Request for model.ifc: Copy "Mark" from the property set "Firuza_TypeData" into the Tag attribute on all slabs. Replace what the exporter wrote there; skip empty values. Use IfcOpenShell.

First a look at what the model holds.

```python
import ifcopenshell
import ifcopenshell.util.element

model = ifcopenshell.open("model.ifc")
print(model.schema)
slabs = model.by_type("IfcSlab")
print(len(slabs), "slabs")
for e in slabs[:8]:
    source = ifcopenshell.util.element.get_pset(e, "Firuza_TypeData", "Mark")
    target = e.Tag
    print(e.id(), repr(source), repr(target), sep=" | ")
```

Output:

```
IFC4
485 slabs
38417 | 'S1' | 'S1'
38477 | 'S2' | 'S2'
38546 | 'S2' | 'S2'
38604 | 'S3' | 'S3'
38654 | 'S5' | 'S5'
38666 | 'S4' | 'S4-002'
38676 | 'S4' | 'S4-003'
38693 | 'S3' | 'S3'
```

```python
import ifcopenshell
import ifcopenshell.util.element

model = ifcopenshell.open("model.ifc")

count = 0
for e in model.by_type("IfcSlab"):
    value = ifcopenshell.util.element.get_pset(e, "Firuza_TypeData", "Mark")
    current = e.Tag
    if not value or not value.strip() or current == value:
        continue
    e.Tag = value
    count += 1

print(count, "slabs updated")

model.write("model_updated.ifc")
```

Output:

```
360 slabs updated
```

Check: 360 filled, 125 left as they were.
